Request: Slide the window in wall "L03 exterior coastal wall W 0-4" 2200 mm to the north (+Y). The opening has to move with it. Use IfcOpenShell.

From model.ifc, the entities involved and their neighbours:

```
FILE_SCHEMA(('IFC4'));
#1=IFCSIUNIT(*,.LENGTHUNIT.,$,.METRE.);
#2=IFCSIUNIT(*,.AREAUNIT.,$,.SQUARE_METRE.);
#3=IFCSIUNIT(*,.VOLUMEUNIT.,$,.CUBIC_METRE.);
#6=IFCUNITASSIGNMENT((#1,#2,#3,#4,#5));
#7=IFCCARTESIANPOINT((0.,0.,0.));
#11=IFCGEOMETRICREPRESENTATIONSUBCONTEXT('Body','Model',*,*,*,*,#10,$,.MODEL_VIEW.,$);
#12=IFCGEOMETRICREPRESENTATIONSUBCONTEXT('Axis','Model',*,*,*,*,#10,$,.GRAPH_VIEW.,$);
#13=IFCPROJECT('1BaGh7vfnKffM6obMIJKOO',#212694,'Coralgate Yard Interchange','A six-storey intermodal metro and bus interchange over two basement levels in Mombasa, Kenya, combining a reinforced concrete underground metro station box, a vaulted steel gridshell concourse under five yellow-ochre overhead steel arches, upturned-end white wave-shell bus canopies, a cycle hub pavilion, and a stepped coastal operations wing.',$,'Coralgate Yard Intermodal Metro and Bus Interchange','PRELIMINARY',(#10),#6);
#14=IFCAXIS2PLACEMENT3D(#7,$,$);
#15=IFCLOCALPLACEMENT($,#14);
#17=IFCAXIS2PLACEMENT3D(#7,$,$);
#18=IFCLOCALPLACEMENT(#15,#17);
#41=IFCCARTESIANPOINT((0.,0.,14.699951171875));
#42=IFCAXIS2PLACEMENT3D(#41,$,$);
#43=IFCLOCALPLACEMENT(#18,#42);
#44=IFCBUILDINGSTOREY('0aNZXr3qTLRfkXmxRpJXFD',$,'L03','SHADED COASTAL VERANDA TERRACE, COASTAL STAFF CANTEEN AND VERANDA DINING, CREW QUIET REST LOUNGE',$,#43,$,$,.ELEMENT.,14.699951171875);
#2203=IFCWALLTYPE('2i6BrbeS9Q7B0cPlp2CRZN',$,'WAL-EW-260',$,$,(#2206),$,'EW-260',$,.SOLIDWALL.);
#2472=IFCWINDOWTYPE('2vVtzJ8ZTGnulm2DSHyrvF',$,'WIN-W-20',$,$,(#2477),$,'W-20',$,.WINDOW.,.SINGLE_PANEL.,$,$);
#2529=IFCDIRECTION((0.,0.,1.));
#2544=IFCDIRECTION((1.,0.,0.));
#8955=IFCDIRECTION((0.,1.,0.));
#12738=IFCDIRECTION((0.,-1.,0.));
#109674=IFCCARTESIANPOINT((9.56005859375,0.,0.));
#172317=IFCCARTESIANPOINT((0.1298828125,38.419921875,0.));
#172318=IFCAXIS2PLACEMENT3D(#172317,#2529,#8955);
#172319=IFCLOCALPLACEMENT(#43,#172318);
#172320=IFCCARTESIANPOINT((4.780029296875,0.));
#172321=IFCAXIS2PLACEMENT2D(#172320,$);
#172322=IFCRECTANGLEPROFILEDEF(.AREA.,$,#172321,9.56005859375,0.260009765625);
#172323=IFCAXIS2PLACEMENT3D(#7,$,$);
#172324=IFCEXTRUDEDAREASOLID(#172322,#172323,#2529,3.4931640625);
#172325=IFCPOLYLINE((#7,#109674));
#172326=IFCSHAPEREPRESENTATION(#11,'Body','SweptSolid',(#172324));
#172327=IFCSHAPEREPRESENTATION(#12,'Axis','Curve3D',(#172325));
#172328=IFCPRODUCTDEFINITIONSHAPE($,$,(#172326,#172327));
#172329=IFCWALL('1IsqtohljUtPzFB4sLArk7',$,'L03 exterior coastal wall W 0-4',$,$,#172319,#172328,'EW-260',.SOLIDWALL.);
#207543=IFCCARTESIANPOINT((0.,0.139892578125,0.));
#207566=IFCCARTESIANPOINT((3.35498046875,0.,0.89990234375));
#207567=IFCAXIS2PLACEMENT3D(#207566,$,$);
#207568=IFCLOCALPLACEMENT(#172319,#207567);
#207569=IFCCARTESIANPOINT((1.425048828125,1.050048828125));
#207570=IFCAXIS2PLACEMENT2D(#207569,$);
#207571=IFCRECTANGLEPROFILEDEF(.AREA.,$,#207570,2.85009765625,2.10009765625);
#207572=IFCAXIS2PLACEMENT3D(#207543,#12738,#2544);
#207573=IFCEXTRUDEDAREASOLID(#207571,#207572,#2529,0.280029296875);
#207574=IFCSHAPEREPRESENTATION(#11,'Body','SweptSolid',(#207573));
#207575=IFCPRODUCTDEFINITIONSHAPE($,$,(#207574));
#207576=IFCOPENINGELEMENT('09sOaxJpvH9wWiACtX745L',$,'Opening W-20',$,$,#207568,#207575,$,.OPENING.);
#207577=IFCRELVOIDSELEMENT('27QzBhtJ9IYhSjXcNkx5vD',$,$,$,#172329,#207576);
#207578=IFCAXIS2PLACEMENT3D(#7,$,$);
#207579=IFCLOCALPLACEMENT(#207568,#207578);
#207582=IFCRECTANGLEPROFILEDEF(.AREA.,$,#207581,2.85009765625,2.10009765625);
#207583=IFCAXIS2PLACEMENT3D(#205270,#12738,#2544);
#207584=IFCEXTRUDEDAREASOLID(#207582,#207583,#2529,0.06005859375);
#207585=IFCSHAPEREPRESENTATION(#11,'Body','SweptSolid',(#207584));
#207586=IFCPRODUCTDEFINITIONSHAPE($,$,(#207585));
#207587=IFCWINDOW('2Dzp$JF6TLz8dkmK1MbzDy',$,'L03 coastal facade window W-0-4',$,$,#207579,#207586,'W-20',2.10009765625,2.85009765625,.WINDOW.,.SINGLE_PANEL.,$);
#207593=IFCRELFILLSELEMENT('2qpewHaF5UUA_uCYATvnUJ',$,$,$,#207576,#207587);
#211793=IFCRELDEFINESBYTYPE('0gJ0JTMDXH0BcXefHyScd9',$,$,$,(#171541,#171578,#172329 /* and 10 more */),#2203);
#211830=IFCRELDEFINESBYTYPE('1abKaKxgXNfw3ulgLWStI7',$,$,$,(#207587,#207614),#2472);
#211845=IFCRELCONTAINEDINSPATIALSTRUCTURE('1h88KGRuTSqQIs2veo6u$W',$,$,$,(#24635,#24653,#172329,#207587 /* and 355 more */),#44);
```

```python
import ifcopenshell
import ifcopenshell.api.geometry
import ifcopenshell.util.placement

model = ifcopenshell.open("model.ifc")

window = model.by_guid("2Dzp$JF6TLz8dkmK1MbzDy")
opening = window.FillsVoids[0].RelatingOpeningElement
wall = opening.VoidsElements[0].RelatingBuildingElement

wall_matrix = ifcopenshell.util.placement.get_local_placement(wall.ObjectPlacement)
shift = wall_matrix[:3, 0] * 2.2
before = ifcopenshell.util.placement.get_local_placement(window.ObjectPlacement)[:3, 3].copy()

# The window is placed relative to its opening, so it follows when the opening moves.
matrix = ifcopenshell.util.placement.get_local_placement(opening.ObjectPlacement)
matrix[:3, 3] += shift
ifcopenshell.api.geometry.edit_object_placement(
    model, product=opening, matrix=matrix, is_si=False, should_transform_children=True
)

after = ifcopenshell.util.placement.get_local_placement(window.ObjectPlacement)[:3, 3]
print("window moved by", (after - before).round(3) + 0.0)

model.write("model_edited.ifc")
```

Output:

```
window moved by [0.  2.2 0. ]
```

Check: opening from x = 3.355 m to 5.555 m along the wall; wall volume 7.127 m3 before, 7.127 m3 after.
